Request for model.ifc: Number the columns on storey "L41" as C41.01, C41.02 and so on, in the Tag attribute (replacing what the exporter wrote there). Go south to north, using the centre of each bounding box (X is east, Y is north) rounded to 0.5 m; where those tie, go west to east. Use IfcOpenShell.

First a look at what the model holds.

```python
import ifcopenshell
import ifcopenshell.util.element
import ifcopenshell.util.placement

model = ifcopenshell.open("model.ifc")
print(model.schema)
storey = next(s for s in model.by_type("IfcBuildingStorey") if s.Name == "L41")
columns = [e for e in ifcopenshell.util.element.get_decomposition(storey) if e.is_a("IfcColumn")]
for e in sorted(columns, key=lambda e: e.id()):
    origin = ifcopenshell.util.placement.get_local_placement(e.ObjectPlacement)[:3, 3]
    print(e.id(), e.Tag, e.Name, origin.round(2) + 0.0, sep=" | ")
```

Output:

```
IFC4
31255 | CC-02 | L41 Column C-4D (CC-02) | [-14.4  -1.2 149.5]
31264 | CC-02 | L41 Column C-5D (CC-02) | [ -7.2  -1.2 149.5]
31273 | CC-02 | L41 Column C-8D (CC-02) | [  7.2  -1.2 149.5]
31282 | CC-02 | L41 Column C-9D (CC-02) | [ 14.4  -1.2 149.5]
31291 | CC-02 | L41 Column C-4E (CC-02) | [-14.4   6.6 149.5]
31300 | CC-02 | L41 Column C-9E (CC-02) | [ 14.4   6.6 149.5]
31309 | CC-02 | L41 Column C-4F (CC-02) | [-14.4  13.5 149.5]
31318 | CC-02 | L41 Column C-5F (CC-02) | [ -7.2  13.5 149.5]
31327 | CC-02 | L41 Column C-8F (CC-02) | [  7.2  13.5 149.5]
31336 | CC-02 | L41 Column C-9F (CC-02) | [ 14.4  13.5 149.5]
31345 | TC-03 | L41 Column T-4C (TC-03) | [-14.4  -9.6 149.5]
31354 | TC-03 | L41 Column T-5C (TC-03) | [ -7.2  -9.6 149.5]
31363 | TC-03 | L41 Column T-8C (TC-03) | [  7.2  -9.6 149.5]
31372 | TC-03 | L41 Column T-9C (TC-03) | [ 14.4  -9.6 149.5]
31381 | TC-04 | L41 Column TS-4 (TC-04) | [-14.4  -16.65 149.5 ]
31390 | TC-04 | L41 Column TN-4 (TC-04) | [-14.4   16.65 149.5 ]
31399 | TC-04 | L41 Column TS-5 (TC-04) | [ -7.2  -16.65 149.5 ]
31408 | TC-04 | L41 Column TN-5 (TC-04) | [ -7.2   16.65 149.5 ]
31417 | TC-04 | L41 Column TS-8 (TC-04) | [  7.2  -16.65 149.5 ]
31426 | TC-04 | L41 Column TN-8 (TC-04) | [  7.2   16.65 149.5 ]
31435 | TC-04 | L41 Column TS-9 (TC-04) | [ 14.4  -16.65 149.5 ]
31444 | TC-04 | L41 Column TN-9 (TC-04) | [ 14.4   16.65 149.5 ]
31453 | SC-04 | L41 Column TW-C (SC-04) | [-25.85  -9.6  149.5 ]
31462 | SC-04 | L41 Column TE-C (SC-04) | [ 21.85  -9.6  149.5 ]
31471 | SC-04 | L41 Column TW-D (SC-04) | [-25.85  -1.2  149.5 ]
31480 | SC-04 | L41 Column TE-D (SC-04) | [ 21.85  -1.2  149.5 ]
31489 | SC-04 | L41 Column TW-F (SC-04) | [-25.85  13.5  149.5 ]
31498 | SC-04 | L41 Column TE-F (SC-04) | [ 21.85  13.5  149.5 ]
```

```python
import ifcopenshell
import ifcopenshell.geom
import ifcopenshell.util.element
import ifcopenshell.util.shape

model = ifcopenshell.open("model.ifc")
settings = ifcopenshell.geom.settings()
settings.set("use-world-coords", True)


def centre(element):
    shape = ifcopenshell.geom.create_shape(settings, element)
    return ifcopenshell.util.shape.get_bbox_centroid(shape.geometry)


storey = next(s for s in model.by_type("IfcBuildingStorey") if s.Name == "L41")
columns = [e for e in ifcopenshell.util.element.get_decomposition(storey) if e.is_a("IfcColumn")]

# Insertion points can sit at a corner or the storey origin, so sort by the geometry (in metres).
centres = {e: centre(e) for e in columns}
columns.sort(key=lambda e: (round(centres[e][1] / 0.5), centres[e][0]))

for i, e in enumerate(columns, start=1):
    number = f"C41.{i:02d}"
    e.Tag = number
    print(e.id(), number)

model.write("model_v2.ifc")
```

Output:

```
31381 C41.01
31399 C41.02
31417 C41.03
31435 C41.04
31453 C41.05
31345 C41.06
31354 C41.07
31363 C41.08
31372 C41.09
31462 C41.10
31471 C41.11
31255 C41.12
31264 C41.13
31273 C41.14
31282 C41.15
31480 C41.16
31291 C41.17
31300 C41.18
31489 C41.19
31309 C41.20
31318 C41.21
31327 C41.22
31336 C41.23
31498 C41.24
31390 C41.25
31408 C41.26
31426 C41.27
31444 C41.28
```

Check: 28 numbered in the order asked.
